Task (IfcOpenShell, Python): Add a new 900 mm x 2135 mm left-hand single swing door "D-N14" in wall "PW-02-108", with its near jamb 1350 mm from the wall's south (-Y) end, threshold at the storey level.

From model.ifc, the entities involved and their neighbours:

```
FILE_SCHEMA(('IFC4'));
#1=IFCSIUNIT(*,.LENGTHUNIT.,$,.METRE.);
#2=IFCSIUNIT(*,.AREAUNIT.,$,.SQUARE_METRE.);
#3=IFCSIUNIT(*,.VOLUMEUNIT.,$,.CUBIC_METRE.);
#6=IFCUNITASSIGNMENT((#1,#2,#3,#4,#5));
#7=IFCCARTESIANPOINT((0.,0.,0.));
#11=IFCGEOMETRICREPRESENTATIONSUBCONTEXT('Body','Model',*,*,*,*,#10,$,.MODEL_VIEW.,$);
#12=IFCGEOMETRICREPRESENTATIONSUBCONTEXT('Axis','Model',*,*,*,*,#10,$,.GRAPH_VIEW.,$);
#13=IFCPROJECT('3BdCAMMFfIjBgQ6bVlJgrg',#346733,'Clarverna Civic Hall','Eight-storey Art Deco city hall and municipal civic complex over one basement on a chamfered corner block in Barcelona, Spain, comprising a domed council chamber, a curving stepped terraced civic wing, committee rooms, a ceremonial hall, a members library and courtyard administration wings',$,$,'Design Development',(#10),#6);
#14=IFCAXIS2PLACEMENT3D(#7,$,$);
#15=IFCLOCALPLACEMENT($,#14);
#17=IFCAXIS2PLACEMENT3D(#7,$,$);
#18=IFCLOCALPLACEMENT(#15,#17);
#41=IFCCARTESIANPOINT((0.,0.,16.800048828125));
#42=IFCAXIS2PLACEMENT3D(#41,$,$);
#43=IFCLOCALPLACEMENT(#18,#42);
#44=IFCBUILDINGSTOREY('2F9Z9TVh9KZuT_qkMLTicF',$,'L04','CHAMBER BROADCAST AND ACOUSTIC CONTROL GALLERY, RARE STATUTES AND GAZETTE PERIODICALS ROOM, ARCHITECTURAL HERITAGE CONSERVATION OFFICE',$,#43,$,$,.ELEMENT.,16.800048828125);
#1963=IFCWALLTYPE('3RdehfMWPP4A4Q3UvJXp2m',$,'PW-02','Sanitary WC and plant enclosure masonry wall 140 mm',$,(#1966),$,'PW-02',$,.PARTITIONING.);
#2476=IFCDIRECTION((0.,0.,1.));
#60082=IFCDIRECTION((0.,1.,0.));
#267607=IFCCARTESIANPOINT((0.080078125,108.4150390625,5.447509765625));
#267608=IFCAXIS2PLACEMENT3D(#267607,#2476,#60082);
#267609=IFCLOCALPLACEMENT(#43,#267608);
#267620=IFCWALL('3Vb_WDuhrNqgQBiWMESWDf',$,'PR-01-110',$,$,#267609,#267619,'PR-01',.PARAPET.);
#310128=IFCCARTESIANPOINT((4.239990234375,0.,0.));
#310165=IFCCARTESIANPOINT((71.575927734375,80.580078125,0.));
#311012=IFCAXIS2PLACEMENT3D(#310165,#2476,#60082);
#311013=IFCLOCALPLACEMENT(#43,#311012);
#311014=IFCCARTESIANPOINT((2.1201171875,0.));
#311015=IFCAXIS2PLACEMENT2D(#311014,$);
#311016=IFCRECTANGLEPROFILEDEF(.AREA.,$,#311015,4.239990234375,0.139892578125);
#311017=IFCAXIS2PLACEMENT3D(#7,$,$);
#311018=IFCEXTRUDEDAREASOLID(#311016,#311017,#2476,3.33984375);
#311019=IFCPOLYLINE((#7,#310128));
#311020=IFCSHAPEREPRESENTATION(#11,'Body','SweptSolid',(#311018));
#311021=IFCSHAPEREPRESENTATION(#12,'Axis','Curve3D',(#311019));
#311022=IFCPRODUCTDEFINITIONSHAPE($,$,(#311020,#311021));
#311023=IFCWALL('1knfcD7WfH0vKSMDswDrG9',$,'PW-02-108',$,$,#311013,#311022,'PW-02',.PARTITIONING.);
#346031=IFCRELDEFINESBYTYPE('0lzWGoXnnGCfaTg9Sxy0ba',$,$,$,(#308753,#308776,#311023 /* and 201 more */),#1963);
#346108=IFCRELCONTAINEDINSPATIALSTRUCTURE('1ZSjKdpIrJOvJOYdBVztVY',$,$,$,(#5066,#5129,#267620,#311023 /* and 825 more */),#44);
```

```python
import numpy as np
import ifcopenshell
import ifcopenshell.api.feature
import ifcopenshell.api.geometry
import ifcopenshell.api.root
import ifcopenshell.api.spatial
import ifcopenshell.geom
import ifcopenshell.util.element
import ifcopenshell.util.placement
import ifcopenshell.util.representation
import ifcopenshell.util.shape
import ifcopenshell.util.unit

model = ifcopenshell.open("model.ifc")
unit_scale = ifcopenshell.util.unit.calculate_unit_scale(model)
settings = ifcopenshell.geom.settings()


def volume(element):
    """Net volume in cubic metres, openings subtracted."""
    shape = ifcopenshell.geom.create_shape(settings, element)
    return ifcopenshell.util.shape.get_volume(shape.geometry)


wall = model.by_guid("1knfcD7WfH0vKSMDswDrG9")
storey = ifcopenshell.util.element.get_container(wall, ifc_class="IfcBuildingStorey")
context = ifcopenshell.util.representation.get_context(model, "Model", "Body", "MODEL_VIEW")
before = volume(wall)

width, height, from_end, sill = 0.9, 2.135, 1.35, 0.0  # metres

# The wall runs along its own X axis, and the end named is its -X end.
wall_shape = ifcopenshell.geom.create_shape(settings, wall)
x, y, z = ifcopenshell.util.shape.get_vertices(wall_shape.geometry).T
start = x.min() + from_end
face, thickness = float(y.min()), float(y.max() - y.min())
wall_matrix = ifcopenshell.util.placement.get_local_placement(wall.ObjectPlacement)
level = ifcopenshell.util.placement.get_local_placement(storey.ObjectPlacement)[2, 3]


def in_wall(x, y):
    """Placement at x, y metres in the wall's axes, at sill height."""
    matrix = wall_matrix.copy()
    matrix[:, 3] = wall_matrix @ np.array([x / unit_scale, y / unit_scale, 0.0, 1.0])
    matrix[2, 3] = level + sill / unit_scale
    return matrix


# Opening: a box that overshoots both wall faces by 50 mm.
opening = ifcopenshell.api.root.create_entity(model, ifc_class="IfcOpeningElement", predefined_type="OPENING")
box = ifcopenshell.api.geometry.add_wall_representation(
    model, context=context, length=width, height=height, thickness=thickness + 0.1
)
ifcopenshell.api.geometry.assign_representation(model, product=opening, representation=box)
ifcopenshell.api.geometry.edit_object_placement(model, product=opening, matrix=in_wall(start, face - 0.05), is_si=False)
ifcopenshell.api.feature.add_feature(model, feature=opening, element=wall)

door = ifcopenshell.api.root.create_entity(model, ifc_class="IfcDoor", name="D-N14", predefined_type="DOOR")
door.OverallWidth, door.OverallHeight = width / unit_scale, height / unit_scale
door.OperationType = "SINGLE_SWING_LEFT"
body = ifcopenshell.api.geometry.add_door_representation(
    model,
    context=context,
    overall_width=door.OverallWidth,
    overall_height=door.OverallHeight,
    operation_type="SINGLE_SWING_LEFT",
    lining_properties={"LiningDepth": thickness / unit_scale, "ThresholdDepth": thickness / unit_scale},
)
ifcopenshell.api.geometry.assign_representation(model, product=door, representation=body)
ifcopenshell.api.spatial.assign_container(model, products=[door], relating_structure=storey)
ifcopenshell.api.feature.add_filling(model, opening=opening, element=door)

# The lining spans the wall, so the door starts at the wall face.
ifcopenshell.api.geometry.edit_object_placement(model, product=door, matrix=in_wall(start, face), is_si=False)

after = volume(wall)

print(f"wall volume {before:.3f} -> {after:.3f} m3")

model.write("model_updated.ifc")
```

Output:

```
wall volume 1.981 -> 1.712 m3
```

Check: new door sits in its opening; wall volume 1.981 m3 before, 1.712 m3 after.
